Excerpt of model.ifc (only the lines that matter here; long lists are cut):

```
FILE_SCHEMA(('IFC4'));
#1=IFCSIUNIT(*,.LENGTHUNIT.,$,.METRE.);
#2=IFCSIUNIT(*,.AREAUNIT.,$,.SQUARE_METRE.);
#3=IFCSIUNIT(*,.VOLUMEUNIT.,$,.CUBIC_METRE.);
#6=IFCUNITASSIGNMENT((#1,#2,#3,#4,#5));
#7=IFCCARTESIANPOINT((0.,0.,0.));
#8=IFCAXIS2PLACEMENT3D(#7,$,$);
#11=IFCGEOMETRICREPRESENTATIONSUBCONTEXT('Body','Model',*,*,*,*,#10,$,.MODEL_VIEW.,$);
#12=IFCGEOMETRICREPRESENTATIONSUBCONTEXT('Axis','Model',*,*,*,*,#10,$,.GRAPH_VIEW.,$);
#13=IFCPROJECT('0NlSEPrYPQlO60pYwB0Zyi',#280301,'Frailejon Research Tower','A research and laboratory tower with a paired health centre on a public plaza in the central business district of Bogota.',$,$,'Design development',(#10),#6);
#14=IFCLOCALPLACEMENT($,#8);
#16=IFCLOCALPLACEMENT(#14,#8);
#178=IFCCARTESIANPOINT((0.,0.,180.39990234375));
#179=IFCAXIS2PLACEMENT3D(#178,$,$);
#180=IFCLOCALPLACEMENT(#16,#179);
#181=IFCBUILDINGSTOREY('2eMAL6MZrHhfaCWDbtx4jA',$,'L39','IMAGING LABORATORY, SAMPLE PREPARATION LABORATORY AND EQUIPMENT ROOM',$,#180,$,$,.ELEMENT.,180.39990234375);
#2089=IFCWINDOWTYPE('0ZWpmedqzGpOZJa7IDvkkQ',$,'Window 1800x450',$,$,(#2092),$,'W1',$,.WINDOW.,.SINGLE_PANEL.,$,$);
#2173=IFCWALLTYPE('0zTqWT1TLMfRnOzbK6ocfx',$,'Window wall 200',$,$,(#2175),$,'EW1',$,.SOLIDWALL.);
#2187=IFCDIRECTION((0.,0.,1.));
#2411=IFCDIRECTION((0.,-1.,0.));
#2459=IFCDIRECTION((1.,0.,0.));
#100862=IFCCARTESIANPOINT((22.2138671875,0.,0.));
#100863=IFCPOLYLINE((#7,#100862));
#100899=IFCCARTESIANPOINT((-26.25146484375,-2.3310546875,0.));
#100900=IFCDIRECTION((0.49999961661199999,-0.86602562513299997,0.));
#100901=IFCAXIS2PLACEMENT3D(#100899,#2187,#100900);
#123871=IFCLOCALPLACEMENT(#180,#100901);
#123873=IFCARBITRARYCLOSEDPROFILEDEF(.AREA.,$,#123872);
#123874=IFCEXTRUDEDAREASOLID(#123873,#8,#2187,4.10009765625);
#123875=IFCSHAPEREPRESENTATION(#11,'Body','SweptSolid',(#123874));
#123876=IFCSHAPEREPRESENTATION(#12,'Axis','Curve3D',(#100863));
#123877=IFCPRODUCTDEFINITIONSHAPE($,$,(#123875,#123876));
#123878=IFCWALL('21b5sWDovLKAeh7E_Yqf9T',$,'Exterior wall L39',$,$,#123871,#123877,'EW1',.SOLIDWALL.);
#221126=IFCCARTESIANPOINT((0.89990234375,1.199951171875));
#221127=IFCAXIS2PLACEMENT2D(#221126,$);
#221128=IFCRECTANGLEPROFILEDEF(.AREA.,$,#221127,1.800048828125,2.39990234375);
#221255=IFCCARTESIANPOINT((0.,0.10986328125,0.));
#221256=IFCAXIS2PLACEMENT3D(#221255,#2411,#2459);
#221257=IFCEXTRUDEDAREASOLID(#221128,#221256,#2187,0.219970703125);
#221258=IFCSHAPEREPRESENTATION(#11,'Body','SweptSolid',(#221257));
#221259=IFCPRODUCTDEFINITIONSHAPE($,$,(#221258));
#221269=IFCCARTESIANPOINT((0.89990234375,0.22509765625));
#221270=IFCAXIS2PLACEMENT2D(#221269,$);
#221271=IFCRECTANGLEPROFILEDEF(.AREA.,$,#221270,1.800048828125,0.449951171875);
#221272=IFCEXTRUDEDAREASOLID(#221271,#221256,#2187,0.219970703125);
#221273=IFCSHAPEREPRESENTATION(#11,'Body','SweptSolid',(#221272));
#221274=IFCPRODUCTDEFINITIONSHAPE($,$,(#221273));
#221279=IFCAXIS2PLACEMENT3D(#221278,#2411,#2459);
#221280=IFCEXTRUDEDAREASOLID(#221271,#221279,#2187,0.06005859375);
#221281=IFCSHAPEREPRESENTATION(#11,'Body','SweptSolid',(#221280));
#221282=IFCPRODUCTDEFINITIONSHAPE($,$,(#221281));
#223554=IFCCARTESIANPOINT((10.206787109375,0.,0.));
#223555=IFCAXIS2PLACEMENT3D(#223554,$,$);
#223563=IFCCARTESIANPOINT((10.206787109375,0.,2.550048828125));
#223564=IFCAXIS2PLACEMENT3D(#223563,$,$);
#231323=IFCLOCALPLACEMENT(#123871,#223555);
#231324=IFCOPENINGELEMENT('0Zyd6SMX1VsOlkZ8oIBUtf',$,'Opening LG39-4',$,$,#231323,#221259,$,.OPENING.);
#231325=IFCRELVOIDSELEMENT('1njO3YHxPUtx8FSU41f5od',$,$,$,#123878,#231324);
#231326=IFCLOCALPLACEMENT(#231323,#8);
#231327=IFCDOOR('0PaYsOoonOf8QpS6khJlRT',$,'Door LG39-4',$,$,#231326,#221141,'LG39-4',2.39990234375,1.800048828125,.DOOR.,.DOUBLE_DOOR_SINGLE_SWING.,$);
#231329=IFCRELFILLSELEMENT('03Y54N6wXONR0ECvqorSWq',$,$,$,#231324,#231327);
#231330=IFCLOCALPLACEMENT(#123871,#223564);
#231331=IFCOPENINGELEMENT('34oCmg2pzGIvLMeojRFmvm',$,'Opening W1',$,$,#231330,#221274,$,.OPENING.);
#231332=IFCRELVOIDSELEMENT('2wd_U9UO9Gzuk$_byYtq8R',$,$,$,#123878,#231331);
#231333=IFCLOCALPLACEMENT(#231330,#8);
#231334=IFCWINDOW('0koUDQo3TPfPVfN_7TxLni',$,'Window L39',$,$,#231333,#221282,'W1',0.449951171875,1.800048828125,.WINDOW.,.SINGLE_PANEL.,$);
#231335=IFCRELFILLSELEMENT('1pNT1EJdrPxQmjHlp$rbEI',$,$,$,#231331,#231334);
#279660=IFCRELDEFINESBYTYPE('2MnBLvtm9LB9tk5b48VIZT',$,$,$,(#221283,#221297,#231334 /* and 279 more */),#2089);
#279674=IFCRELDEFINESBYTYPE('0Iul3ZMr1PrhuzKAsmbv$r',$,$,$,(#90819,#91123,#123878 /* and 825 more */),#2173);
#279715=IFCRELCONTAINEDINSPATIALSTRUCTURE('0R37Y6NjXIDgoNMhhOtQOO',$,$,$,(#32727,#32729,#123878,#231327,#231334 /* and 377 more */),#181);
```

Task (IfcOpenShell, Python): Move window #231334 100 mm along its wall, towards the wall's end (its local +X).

```python
import ifcopenshell
import ifcopenshell.api.geometry
import ifcopenshell.util.placement

model = ifcopenshell.open("model.ifc")

window = model.by_guid("0koUDQo3TPfPVfN_7TxLni")
opening = window.FillsVoids[0].RelatingOpeningElement
wall = opening.VoidsElements[0].RelatingBuildingElement

wall_matrix = ifcopenshell.util.placement.get_local_placement(wall.ObjectPlacement)
shift = wall_matrix[:3, 0] * 0.1
before = ifcopenshell.util.placement.get_local_placement(window.ObjectPlacement)[:3, 3].copy()

# The window is placed relative to its opening, so it follows when the opening moves.
matrix = ifcopenshell.util.placement.get_local_placement(opening.ObjectPlacement)
matrix[:3, 3] += shift
ifcopenshell.api.geometry.edit_object_placement(
    model, product=opening, matrix=matrix, is_si=False, should_transform_children=True
)

after = ifcopenshell.util.placement.get_local_placement(window.ObjectPlacement)[:3, 3]
print("window moved by", (after - before).round(3) + 0.0)

model.write("model_edited.ifc")
```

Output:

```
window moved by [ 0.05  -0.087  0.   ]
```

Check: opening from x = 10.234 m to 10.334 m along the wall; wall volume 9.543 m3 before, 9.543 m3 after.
